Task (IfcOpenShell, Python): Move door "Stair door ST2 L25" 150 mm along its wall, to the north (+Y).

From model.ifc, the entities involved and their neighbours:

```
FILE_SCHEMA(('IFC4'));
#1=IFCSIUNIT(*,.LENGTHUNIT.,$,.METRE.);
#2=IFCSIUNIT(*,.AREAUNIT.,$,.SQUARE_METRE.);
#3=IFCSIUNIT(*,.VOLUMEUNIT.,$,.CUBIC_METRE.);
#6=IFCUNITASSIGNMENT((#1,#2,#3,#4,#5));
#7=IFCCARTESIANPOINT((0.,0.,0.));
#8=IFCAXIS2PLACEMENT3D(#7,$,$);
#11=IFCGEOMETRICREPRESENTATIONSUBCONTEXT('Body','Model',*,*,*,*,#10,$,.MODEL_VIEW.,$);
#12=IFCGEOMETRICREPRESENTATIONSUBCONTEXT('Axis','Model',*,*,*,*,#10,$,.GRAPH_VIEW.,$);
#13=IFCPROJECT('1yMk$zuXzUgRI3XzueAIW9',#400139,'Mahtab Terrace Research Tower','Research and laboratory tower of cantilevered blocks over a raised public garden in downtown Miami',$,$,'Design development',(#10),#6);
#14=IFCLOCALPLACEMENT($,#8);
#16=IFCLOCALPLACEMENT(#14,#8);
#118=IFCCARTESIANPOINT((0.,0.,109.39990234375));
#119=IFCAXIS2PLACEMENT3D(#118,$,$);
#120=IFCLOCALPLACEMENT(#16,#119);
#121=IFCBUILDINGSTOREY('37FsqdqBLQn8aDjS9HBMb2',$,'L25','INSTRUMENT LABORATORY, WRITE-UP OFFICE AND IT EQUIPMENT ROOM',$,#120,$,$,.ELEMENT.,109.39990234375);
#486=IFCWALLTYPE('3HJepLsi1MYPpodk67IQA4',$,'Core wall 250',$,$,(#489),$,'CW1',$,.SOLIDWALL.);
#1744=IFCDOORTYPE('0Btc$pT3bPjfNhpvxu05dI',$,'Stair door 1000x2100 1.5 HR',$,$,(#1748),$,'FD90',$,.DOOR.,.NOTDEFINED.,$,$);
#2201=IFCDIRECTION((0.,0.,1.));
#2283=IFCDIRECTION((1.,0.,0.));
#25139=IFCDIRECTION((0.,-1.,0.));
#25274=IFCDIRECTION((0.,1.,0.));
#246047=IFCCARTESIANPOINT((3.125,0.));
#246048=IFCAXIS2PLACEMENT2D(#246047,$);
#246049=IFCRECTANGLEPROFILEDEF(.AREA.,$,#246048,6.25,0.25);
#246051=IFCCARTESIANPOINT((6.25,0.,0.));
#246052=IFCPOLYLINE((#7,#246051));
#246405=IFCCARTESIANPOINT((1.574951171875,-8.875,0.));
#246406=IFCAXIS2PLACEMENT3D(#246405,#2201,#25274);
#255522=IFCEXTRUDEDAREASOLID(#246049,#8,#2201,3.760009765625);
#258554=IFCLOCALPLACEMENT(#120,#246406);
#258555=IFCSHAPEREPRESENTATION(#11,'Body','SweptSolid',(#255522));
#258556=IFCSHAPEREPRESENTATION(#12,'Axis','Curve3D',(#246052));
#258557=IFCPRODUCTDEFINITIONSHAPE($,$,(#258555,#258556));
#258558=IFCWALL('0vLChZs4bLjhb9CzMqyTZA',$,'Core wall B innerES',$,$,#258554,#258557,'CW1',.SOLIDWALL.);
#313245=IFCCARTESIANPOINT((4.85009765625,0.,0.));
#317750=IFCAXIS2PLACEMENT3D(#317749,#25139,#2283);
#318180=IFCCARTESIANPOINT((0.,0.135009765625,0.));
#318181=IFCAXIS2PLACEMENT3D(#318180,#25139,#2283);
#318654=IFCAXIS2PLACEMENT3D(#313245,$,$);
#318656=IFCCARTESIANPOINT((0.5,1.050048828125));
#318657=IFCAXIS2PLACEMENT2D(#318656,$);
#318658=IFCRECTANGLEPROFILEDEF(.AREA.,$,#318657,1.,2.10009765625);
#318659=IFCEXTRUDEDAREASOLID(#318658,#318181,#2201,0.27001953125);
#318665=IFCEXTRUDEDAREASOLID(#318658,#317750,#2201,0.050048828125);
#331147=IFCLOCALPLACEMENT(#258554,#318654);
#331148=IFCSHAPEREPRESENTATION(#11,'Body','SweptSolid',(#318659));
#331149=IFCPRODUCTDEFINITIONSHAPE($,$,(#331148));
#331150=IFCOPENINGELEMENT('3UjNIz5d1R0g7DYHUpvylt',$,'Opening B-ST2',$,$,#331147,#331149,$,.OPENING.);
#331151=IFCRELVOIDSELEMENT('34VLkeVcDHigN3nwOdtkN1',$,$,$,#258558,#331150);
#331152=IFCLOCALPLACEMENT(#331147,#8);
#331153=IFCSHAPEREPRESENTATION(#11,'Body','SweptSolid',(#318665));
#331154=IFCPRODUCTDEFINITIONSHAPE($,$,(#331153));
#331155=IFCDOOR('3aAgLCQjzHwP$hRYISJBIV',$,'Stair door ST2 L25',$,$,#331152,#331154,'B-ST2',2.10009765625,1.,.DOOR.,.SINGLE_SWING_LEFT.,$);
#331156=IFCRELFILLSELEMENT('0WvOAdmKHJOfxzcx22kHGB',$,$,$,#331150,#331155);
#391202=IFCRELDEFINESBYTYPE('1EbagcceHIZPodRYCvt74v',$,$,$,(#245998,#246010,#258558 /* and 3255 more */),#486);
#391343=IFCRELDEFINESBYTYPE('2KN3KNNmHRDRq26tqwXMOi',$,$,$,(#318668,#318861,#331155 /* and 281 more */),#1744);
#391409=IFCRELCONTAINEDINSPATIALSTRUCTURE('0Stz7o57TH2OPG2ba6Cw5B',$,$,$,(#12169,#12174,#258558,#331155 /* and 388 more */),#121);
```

```python
import ifcopenshell
import ifcopenshell.api.geometry
import ifcopenshell.util.placement
import ifcopenshell.util.unit

model = ifcopenshell.open("model.ifc")
unit_scale = ifcopenshell.util.unit.calculate_unit_scale(model)

door = model.by_guid("3aAgLCQjzHwP$hRYISJBIV")
opening = door.FillsVoids[0].RelatingOpeningElement
wall = opening.VoidsElements[0].RelatingBuildingElement

wall_matrix = ifcopenshell.util.placement.get_local_placement(wall.ObjectPlacement)
shift = wall_matrix[:3, 0] * 0.15 / unit_scale
before = ifcopenshell.util.placement.get_local_placement(door.ObjectPlacement)[:3, 3].copy()

# The door is placed relative to its opening, so it follows when the opening moves.
matrix = ifcopenshell.util.placement.get_local_placement(opening.ObjectPlacement)
matrix[:3, 3] += shift
ifcopenshell.api.geometry.edit_object_placement(
    model, product=opening, matrix=matrix, is_si=False, should_transform_children=True
)

after = ifcopenshell.util.placement.get_local_placement(door.ObjectPlacement)[:3, 3]
print("door moved by", (after - before).round(3) + 0.0)

model.write("model_edited.ifc")
```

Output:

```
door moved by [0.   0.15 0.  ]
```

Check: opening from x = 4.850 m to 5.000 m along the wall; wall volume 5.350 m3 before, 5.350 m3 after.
